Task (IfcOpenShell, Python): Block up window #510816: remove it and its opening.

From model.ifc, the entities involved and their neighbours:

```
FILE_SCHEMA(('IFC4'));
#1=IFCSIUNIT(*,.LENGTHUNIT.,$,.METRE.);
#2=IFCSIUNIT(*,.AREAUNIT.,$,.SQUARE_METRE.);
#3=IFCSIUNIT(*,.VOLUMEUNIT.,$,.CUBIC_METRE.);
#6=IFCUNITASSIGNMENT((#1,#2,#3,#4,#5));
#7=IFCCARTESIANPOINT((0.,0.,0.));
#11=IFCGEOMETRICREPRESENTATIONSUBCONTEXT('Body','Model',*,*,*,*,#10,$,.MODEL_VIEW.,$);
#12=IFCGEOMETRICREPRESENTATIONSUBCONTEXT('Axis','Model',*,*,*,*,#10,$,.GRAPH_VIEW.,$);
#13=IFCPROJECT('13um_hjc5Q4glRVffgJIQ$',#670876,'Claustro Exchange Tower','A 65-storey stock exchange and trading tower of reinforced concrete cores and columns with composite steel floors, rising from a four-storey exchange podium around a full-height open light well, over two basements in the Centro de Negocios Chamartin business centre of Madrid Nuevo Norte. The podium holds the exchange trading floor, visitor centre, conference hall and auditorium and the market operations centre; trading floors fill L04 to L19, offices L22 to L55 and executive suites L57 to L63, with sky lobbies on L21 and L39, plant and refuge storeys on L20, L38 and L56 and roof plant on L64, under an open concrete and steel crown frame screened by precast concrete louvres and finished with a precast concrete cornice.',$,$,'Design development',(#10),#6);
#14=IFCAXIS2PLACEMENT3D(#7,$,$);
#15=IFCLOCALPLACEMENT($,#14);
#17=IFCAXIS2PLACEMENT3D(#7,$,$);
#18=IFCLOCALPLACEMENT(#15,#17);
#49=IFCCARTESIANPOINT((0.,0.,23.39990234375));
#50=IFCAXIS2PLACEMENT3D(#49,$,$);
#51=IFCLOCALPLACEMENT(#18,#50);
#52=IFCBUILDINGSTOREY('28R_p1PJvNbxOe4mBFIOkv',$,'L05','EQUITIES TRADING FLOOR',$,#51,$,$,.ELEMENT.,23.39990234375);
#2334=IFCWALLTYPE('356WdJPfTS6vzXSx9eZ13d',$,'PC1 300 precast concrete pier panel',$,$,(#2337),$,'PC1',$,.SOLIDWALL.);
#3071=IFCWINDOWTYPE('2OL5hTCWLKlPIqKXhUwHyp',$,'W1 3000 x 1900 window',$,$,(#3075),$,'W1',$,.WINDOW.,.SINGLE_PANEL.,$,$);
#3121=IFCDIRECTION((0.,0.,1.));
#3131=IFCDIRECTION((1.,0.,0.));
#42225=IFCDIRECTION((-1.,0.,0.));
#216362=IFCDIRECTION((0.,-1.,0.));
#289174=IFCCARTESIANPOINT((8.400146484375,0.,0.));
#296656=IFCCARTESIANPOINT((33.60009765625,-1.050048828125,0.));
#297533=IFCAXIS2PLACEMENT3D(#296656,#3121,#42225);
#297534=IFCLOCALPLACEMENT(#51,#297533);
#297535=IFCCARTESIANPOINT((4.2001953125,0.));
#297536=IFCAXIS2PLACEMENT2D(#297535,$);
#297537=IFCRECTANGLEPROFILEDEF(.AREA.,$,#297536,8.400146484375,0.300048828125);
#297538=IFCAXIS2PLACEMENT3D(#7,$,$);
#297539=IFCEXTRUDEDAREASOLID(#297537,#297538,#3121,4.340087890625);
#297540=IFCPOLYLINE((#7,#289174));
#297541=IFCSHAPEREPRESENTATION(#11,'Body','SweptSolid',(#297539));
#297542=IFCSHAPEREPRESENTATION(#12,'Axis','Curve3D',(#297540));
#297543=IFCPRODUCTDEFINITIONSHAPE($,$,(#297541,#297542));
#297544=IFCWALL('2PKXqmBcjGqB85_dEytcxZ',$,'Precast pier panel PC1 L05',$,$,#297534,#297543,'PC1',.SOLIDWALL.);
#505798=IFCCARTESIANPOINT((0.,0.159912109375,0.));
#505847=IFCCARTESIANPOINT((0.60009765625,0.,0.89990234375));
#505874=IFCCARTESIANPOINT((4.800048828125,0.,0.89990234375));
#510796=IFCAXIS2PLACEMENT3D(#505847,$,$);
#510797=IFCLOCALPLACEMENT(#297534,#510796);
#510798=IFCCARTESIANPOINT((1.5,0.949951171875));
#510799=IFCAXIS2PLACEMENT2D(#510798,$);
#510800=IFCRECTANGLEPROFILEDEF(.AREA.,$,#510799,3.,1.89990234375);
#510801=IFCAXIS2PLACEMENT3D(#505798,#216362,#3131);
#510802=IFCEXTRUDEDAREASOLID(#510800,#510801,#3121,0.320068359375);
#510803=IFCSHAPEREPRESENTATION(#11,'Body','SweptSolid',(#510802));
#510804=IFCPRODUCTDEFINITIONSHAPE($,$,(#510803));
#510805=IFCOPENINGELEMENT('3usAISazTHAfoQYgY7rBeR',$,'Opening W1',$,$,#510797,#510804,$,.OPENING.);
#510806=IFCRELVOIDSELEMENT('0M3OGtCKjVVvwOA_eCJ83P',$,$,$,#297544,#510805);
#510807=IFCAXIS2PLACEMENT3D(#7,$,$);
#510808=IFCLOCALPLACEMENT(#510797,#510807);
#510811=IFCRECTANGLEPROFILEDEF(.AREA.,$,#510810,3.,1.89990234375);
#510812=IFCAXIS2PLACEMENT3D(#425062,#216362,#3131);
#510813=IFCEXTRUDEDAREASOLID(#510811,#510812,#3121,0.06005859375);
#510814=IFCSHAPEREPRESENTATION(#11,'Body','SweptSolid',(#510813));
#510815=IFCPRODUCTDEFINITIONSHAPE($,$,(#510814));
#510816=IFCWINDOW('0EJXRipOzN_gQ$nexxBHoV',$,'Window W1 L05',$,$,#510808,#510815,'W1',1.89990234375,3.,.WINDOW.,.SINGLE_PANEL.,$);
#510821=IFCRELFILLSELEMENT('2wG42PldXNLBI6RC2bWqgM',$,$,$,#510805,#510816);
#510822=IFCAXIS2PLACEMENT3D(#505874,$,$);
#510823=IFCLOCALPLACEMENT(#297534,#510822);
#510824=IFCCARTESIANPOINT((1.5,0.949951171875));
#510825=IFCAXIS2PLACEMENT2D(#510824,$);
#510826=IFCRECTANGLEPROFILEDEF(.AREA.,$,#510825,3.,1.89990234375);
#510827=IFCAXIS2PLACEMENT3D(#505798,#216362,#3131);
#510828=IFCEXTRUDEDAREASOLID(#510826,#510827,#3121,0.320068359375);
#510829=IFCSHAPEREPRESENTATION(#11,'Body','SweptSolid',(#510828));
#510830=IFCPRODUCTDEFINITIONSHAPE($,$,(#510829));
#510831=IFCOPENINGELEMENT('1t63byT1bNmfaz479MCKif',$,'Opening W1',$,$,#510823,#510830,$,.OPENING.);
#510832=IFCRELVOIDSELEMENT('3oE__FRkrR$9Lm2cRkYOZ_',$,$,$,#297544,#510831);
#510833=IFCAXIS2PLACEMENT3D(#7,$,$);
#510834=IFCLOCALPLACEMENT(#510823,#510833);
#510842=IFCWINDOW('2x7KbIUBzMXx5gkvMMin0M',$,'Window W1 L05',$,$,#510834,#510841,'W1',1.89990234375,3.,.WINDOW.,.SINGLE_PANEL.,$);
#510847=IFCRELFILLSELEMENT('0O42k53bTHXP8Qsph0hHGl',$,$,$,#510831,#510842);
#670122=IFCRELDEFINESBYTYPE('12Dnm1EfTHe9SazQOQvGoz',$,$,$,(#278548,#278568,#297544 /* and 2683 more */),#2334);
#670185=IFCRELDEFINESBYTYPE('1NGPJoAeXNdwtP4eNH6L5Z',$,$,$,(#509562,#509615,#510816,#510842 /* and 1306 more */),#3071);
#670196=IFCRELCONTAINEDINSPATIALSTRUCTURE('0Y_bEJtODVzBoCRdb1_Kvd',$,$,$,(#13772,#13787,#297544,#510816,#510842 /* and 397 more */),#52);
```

```python
import ifcopenshell
import ifcopenshell.api.feature
import ifcopenshell.api.root
import ifcopenshell.geom
import ifcopenshell.util.shape

model = ifcopenshell.open("model.ifc")
settings = ifcopenshell.geom.settings()


def volume(element):
    """Net volume in cubic metres, openings subtracted."""
    shape = ifcopenshell.geom.create_shape(settings, element)
    return ifcopenshell.util.shape.get_volume(shape.geometry)


window = model.by_guid("0EJXRipOzN_gQ$nexxBHoV")
opening = window.FillsVoids[0].RelatingOpeningElement
wall = opening.VoidsElements[0].RelatingBuildingElement
before = volume(wall)

ifcopenshell.api.root.remove_product(model, product=window)
ifcopenshell.api.feature.remove_feature(model, feature=opening)

after = volume(wall)

print(f"wall volume {before:.3f} -> {after:.3f} m3")

model.write("model_v2.ifc")
```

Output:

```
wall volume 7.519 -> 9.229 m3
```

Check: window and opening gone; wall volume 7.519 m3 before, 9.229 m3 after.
